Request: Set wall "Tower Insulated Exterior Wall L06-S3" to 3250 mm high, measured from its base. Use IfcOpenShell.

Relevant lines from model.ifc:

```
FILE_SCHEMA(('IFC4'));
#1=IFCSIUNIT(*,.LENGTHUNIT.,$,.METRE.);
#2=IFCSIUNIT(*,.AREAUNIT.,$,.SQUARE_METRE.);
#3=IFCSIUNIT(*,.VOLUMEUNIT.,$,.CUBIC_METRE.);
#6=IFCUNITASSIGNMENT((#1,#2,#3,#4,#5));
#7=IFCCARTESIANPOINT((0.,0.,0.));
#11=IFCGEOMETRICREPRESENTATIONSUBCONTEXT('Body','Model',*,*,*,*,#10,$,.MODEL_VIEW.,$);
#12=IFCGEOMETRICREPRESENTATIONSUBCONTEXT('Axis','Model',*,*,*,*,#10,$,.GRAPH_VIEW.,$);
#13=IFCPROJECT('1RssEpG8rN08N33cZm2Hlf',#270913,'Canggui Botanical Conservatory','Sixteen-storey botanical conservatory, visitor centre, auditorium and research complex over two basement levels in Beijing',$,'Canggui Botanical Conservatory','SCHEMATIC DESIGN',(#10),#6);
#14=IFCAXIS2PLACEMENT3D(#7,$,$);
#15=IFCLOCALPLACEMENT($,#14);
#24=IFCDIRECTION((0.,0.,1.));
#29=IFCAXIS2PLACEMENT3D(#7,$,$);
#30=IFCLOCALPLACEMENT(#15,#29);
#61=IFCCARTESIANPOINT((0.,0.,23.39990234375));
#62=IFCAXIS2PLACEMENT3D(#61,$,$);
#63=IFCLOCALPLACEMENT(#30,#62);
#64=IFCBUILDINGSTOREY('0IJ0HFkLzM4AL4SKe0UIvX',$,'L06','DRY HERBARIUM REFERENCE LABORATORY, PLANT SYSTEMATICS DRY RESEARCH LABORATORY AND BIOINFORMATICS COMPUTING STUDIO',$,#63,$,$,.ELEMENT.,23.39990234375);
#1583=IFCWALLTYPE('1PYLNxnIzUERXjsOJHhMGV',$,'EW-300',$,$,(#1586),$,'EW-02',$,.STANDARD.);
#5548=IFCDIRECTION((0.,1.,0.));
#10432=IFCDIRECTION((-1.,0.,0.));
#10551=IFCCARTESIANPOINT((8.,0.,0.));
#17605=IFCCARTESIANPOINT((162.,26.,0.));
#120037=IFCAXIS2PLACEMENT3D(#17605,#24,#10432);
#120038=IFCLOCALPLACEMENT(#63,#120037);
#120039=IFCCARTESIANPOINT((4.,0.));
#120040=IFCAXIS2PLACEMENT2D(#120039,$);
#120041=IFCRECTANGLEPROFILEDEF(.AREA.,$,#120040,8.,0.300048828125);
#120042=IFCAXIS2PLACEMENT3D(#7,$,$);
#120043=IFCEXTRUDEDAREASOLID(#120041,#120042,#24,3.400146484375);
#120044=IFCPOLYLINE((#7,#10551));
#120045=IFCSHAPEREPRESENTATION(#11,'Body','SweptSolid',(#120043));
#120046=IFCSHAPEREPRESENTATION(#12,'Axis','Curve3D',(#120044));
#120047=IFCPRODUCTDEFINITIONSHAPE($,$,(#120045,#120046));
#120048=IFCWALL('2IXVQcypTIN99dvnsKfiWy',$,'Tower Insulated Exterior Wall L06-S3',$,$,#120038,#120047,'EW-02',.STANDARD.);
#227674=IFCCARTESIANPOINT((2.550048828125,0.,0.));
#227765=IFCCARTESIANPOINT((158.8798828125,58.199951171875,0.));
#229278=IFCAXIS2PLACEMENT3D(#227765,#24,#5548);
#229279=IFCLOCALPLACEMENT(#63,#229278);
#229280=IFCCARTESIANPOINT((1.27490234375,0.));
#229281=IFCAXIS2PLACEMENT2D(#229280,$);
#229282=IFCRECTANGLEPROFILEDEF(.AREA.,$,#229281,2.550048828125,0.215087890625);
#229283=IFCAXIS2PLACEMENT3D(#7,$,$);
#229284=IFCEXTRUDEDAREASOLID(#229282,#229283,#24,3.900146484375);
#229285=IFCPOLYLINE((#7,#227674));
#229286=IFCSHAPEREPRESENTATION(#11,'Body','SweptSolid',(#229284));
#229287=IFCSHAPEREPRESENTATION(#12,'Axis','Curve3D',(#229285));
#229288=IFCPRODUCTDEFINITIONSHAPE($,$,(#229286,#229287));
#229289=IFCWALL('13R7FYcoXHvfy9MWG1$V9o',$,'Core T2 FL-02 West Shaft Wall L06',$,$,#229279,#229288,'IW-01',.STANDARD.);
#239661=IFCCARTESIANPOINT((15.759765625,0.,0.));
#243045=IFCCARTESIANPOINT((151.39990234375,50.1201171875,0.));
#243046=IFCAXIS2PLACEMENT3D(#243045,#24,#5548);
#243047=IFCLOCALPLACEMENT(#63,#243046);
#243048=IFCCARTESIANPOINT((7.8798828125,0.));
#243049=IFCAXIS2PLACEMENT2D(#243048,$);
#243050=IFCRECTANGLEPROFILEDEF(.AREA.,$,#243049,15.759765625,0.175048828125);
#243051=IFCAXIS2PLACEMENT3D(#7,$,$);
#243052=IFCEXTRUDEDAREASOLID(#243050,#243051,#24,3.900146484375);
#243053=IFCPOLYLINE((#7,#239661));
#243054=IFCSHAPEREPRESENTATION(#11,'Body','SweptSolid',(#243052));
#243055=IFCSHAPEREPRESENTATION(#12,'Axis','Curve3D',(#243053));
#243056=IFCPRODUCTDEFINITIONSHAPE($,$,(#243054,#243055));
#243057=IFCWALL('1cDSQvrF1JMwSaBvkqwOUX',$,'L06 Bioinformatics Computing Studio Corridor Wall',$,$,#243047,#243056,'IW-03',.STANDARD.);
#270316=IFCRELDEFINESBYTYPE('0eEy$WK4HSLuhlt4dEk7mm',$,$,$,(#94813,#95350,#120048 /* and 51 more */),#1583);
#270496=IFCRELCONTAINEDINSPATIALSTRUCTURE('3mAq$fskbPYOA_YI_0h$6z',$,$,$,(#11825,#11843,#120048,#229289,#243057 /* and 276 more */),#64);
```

```python
import ifcopenshell
import ifcopenshell.geom
import ifcopenshell.util.representation
import ifcopenshell.util.shape
import ifcopenshell.util.unit

model = ifcopenshell.open("model.ifc")
unit_scale = ifcopenshell.util.unit.calculate_unit_scale(model)
settings = ifcopenshell.geom.settings()


def volume(element):
    """Net volume in cubic metres, openings subtracted."""
    shape = ifcopenshell.geom.create_shape(settings, element)
    return ifcopenshell.util.shape.get_volume(shape.geometry)


wall = model.by_guid("2IXVQcypTIN99dvnsKfiWy")
before = volume(wall)

body = ifcopenshell.util.representation.get_representation(wall, "Model", "Body")
solid = body.Items[0]
old_height = solid.Depth
solid.Depth = 3.25 / unit_scale
after = volume(wall)

print(f"height {old_height:g} -> {solid.Depth:g}, volume {before:.3f} -> {after:.3f} m3")

model.write("model_edited.ifc")
```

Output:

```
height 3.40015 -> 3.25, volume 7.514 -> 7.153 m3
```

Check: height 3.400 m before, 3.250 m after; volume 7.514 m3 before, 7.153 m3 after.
